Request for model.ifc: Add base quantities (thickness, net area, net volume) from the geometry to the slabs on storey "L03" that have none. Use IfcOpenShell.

First a look at what the model holds.

```python
import ifcopenshell
import ifcopenshell.util.element
import ifcopenshell.util.unit

model = ifcopenshell.open("model.ifc")
print(model.schema)
for unit_type in ("LENGTHUNIT", "AREAUNIT", "VOLUMEUNIT"):
    print(unit_type, ifcopenshell.util.unit.calculate_unit_scale(model, unit_type))
storey = next(s for s in model.by_type("IfcBuildingStorey") if s.Name == "L03")
slabs = [e for e in ifcopenshell.util.element.get_decomposition(storey) if e.is_a("IfcSlab")]
for e in sorted(slabs, key=lambda e: e.id()):
    print(e.id(), e.is_a(), e.Name, list(ifcopenshell.util.element.get_psets(e, qtos_only=True)), sep=" | ")
```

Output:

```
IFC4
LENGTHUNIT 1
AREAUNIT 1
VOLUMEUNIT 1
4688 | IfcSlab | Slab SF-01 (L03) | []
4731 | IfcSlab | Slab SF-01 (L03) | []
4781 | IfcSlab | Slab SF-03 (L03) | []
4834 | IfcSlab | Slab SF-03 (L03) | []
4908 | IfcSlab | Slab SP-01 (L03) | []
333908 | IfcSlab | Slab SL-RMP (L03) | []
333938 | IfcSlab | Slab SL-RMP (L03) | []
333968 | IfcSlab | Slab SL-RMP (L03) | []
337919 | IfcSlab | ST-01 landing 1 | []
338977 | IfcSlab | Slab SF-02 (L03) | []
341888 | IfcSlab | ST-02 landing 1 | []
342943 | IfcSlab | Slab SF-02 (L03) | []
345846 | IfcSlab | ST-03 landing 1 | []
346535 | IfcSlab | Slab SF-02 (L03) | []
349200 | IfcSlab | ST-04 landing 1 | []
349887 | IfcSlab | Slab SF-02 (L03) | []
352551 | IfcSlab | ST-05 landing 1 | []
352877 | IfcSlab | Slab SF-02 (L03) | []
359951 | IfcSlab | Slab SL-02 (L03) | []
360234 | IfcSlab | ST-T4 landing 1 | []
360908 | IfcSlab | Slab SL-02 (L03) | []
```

```python
import ifcopenshell
import ifcopenshell.api.pset
import ifcopenshell.geom
import ifcopenshell.util.element
import ifcopenshell.util.shape
import ifcopenshell.util.unit

model = ifcopenshell.open("model.ifc")
unit_scale = ifcopenshell.util.unit.calculate_unit_scale(model)
area_scale = ifcopenshell.util.unit.calculate_unit_scale(model, "AREAUNIT")
volume_scale = ifcopenshell.util.unit.calculate_unit_scale(model, "VOLUMEUNIT")
settings = ifcopenshell.geom.settings()

storey = next(s for s in model.by_type("IfcBuildingStorey") if s.Name == "L03")
slabs = [e for e in ifcopenshell.util.element.get_decomposition(storey) if e.is_a("IfcSlab")]

for e in sorted(slabs, key=lambda e: e.id()):
    if ifcopenshell.util.element.get_psets(e, qtos_only=True, should_inherit=False):
        continue
    # Geometry comes back in metres, in the element's own axes.
    shape = ifcopenshell.geom.create_shape(settings, e)
    values = {
        "Width": ifcopenshell.util.shape.get_z(shape.geometry) / unit_scale,
        "NetArea": ifcopenshell.util.shape.get_footprint_area(shape.geometry) / area_scale,
        "NetVolume": ifcopenshell.util.shape.get_volume(shape.geometry) / volume_scale,
    }
    qto = ifcopenshell.api.pset.add_qto(model, product=e, name="Qto_SlabBaseQuantities")
    ifcopenshell.api.pset.edit_qto(model, qto=qto, properties=values)
    print(e.id(), {k: round(v, 3) for k, v in values.items()})

model.write("model_edited.ifc")
```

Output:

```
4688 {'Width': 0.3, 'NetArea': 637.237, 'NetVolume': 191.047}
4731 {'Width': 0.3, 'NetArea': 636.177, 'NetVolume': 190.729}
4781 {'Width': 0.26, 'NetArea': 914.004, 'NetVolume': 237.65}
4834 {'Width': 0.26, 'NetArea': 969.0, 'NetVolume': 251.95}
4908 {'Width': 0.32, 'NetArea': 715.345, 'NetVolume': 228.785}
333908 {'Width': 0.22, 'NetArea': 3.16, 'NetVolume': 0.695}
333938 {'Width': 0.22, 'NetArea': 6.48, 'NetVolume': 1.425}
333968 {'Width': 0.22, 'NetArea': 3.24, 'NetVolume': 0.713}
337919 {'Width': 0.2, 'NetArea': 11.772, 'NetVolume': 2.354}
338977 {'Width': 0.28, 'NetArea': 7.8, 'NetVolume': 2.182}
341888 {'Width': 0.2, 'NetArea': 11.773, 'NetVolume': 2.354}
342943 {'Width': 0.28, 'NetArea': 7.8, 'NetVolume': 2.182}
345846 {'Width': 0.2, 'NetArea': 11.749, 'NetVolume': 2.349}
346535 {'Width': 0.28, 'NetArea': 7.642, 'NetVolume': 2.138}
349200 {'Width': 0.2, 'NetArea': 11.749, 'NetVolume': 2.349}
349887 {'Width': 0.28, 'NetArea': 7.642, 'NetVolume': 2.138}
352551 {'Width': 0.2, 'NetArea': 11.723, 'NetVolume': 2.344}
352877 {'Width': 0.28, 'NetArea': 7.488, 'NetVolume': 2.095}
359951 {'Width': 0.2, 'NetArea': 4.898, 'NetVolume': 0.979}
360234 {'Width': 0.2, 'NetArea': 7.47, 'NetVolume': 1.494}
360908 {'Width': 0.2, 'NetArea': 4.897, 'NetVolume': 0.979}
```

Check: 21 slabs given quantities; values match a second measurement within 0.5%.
